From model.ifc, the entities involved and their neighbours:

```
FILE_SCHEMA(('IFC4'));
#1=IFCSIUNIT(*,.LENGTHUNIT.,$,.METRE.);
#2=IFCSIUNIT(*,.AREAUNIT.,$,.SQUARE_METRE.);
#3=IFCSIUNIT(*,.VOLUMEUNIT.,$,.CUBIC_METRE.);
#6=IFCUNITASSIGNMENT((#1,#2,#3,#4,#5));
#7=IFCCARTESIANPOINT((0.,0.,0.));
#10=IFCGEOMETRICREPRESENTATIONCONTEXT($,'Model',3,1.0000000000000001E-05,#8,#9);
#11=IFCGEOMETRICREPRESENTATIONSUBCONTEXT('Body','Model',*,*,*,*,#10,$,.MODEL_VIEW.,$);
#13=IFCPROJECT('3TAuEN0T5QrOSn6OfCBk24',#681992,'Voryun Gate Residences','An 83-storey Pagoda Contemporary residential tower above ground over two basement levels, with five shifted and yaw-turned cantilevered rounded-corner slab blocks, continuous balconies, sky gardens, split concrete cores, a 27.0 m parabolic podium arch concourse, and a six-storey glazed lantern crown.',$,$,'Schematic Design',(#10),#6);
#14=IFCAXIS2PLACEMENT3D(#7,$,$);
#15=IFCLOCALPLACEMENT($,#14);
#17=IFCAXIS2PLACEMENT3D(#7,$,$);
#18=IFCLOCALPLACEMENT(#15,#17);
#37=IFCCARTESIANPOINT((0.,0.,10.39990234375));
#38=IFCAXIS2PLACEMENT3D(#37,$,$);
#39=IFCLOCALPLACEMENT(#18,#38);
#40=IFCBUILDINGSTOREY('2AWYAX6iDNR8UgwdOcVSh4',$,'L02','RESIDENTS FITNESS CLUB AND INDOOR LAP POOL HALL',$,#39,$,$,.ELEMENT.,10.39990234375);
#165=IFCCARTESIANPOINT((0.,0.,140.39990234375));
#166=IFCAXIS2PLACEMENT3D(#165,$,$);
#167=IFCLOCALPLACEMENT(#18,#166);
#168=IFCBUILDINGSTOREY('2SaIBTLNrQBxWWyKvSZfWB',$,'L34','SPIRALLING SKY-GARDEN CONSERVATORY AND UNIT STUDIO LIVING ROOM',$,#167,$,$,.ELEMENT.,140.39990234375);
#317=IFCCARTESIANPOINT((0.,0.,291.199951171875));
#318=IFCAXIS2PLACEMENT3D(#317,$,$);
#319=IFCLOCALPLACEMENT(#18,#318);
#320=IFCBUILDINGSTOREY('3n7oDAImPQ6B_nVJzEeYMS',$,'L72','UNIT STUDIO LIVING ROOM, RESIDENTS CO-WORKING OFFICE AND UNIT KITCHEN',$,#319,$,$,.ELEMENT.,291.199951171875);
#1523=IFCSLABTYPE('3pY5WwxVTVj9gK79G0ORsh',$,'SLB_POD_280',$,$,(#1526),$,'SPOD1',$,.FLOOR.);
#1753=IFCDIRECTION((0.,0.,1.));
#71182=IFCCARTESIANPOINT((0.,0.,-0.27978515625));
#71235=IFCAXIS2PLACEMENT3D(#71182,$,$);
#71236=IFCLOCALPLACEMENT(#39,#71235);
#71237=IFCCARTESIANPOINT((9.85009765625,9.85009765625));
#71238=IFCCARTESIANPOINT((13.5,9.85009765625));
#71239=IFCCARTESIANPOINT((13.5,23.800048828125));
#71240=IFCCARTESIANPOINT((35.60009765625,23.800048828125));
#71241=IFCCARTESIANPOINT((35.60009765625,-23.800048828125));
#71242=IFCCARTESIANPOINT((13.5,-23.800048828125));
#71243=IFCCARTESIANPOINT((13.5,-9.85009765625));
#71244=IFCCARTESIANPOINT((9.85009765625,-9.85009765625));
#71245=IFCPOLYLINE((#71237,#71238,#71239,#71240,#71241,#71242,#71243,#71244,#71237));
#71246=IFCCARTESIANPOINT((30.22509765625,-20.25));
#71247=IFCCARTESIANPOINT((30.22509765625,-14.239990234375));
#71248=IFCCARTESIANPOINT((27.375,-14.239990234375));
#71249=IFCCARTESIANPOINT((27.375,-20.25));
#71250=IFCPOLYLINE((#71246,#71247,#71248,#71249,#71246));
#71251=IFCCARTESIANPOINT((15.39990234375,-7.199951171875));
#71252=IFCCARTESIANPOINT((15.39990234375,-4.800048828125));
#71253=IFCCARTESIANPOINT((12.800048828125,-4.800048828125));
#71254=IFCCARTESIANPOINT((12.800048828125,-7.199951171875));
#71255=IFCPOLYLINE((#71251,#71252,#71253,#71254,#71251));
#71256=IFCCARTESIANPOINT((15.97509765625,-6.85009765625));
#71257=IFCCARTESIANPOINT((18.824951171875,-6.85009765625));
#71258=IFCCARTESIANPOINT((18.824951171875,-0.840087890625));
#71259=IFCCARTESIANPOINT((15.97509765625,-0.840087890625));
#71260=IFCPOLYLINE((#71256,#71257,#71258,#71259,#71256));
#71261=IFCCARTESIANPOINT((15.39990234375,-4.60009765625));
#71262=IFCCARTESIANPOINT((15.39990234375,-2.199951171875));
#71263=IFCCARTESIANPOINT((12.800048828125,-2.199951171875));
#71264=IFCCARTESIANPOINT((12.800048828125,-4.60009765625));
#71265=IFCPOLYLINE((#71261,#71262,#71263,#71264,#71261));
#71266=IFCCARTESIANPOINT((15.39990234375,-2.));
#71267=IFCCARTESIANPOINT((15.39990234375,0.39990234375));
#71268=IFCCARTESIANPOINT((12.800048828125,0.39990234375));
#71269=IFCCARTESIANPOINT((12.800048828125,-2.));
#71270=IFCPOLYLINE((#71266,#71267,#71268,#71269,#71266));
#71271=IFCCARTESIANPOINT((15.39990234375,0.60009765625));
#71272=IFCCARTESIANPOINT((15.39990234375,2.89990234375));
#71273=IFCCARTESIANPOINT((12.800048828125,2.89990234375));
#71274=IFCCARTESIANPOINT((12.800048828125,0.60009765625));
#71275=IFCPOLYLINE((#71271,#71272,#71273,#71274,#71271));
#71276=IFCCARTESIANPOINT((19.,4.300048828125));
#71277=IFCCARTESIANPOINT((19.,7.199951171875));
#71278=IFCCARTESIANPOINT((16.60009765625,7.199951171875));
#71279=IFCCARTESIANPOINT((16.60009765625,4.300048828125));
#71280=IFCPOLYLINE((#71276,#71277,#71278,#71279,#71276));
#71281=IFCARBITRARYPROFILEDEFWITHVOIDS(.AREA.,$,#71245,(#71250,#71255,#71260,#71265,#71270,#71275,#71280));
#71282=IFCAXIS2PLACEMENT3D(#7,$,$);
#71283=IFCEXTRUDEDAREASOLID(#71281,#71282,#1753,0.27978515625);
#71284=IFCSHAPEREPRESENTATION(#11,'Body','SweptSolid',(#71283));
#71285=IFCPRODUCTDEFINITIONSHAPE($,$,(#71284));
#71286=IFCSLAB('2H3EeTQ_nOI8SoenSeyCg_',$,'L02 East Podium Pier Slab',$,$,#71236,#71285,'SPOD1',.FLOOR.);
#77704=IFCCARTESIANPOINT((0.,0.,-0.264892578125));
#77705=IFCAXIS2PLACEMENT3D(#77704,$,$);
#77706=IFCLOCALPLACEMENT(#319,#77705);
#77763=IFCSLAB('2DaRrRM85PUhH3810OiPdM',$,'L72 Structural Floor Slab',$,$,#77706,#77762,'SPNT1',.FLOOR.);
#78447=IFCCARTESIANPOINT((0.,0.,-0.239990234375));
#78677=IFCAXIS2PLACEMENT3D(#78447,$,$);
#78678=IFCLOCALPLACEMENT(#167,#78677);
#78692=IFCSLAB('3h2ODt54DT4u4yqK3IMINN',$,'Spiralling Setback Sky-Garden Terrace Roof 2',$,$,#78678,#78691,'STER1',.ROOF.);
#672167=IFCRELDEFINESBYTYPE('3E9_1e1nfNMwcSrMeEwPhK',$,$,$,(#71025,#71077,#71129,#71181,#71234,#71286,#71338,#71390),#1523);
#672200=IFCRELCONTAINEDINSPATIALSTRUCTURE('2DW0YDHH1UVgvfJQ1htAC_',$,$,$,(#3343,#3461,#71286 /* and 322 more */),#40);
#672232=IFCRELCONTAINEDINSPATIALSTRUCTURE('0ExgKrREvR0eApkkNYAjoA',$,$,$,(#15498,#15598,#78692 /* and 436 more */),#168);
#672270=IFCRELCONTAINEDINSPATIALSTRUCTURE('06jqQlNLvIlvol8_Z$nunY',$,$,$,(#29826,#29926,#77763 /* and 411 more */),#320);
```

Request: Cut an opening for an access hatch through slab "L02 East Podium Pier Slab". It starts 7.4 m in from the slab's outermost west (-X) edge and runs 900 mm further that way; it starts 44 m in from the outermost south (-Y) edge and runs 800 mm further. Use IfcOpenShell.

```python
import numpy as np
import ifcopenshell
import ifcopenshell.api.feature
import ifcopenshell.api.geometry
import ifcopenshell.api.root
import ifcopenshell.geom
import ifcopenshell.util.placement
import ifcopenshell.util.representation
import ifcopenshell.util.shape
import ifcopenshell.util.unit

model = ifcopenshell.open("model.ifc")
unit_scale = ifcopenshell.util.unit.calculate_unit_scale(model)
settings = ifcopenshell.geom.settings()


def volume(element):
    """Net volume in cubic metres, openings subtracted."""
    shape = ifcopenshell.geom.create_shape(settings, element)
    return ifcopenshell.util.shape.get_volume(shape.geometry)


slab = model.by_guid("2H3EeTQ_nOI8SoenSeyCg_")
before = volume(slab)

# Extent in the slab's own axes, in metres. The edges named are its -X and -Y sides.
slab_shape = ifcopenshell.geom.create_shape(settings, slab)
vertices = ifcopenshell.util.shape.get_vertices(slab_shape.geometry)
x_min, y_min, bottom = vertices.min(axis=0)
top = vertices[:, 2].max()

opening = ifcopenshell.api.root.create_entity(model, ifc_class="IfcOpeningElement", name="Access hatch opening", predefined_type="OPENING")
context = ifcopenshell.util.representation.get_context(model, "Model", "Body", "MODEL_VIEW")
width, depth = 0.9, 0.8
outline = [(0.0, 0.0), (width, 0.0), (width, depth), (0.0, depth), (0.0, 0.0)]
# Overshoot both faces by 50 mm so the cut is clean.
shape = ifcopenshell.api.geometry.add_slab_representation(
    model, context=context, depth=top - bottom + 0.1, polyline=outline
)
ifcopenshell.api.geometry.assign_representation(model, product=opening, representation=shape)

matrix = ifcopenshell.util.placement.get_local_placement(slab.ObjectPlacement)
matrix[:, 3] = matrix @ np.append(np.array([x_min + 7.4, y_min + 44, bottom - 0.05]) / unit_scale, 1.0)
ifcopenshell.api.geometry.edit_object_placement(model, product=opening, matrix=matrix, is_si=False)
ifcopenshell.api.feature.add_feature(model, feature=opening, element=slab)

after = volume(slab)

print(f"slab volume {before:.3f} -> {after:.3f} m3")

model.write("model_edited.ifc")
```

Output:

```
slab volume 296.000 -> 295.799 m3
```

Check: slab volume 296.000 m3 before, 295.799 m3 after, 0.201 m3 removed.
